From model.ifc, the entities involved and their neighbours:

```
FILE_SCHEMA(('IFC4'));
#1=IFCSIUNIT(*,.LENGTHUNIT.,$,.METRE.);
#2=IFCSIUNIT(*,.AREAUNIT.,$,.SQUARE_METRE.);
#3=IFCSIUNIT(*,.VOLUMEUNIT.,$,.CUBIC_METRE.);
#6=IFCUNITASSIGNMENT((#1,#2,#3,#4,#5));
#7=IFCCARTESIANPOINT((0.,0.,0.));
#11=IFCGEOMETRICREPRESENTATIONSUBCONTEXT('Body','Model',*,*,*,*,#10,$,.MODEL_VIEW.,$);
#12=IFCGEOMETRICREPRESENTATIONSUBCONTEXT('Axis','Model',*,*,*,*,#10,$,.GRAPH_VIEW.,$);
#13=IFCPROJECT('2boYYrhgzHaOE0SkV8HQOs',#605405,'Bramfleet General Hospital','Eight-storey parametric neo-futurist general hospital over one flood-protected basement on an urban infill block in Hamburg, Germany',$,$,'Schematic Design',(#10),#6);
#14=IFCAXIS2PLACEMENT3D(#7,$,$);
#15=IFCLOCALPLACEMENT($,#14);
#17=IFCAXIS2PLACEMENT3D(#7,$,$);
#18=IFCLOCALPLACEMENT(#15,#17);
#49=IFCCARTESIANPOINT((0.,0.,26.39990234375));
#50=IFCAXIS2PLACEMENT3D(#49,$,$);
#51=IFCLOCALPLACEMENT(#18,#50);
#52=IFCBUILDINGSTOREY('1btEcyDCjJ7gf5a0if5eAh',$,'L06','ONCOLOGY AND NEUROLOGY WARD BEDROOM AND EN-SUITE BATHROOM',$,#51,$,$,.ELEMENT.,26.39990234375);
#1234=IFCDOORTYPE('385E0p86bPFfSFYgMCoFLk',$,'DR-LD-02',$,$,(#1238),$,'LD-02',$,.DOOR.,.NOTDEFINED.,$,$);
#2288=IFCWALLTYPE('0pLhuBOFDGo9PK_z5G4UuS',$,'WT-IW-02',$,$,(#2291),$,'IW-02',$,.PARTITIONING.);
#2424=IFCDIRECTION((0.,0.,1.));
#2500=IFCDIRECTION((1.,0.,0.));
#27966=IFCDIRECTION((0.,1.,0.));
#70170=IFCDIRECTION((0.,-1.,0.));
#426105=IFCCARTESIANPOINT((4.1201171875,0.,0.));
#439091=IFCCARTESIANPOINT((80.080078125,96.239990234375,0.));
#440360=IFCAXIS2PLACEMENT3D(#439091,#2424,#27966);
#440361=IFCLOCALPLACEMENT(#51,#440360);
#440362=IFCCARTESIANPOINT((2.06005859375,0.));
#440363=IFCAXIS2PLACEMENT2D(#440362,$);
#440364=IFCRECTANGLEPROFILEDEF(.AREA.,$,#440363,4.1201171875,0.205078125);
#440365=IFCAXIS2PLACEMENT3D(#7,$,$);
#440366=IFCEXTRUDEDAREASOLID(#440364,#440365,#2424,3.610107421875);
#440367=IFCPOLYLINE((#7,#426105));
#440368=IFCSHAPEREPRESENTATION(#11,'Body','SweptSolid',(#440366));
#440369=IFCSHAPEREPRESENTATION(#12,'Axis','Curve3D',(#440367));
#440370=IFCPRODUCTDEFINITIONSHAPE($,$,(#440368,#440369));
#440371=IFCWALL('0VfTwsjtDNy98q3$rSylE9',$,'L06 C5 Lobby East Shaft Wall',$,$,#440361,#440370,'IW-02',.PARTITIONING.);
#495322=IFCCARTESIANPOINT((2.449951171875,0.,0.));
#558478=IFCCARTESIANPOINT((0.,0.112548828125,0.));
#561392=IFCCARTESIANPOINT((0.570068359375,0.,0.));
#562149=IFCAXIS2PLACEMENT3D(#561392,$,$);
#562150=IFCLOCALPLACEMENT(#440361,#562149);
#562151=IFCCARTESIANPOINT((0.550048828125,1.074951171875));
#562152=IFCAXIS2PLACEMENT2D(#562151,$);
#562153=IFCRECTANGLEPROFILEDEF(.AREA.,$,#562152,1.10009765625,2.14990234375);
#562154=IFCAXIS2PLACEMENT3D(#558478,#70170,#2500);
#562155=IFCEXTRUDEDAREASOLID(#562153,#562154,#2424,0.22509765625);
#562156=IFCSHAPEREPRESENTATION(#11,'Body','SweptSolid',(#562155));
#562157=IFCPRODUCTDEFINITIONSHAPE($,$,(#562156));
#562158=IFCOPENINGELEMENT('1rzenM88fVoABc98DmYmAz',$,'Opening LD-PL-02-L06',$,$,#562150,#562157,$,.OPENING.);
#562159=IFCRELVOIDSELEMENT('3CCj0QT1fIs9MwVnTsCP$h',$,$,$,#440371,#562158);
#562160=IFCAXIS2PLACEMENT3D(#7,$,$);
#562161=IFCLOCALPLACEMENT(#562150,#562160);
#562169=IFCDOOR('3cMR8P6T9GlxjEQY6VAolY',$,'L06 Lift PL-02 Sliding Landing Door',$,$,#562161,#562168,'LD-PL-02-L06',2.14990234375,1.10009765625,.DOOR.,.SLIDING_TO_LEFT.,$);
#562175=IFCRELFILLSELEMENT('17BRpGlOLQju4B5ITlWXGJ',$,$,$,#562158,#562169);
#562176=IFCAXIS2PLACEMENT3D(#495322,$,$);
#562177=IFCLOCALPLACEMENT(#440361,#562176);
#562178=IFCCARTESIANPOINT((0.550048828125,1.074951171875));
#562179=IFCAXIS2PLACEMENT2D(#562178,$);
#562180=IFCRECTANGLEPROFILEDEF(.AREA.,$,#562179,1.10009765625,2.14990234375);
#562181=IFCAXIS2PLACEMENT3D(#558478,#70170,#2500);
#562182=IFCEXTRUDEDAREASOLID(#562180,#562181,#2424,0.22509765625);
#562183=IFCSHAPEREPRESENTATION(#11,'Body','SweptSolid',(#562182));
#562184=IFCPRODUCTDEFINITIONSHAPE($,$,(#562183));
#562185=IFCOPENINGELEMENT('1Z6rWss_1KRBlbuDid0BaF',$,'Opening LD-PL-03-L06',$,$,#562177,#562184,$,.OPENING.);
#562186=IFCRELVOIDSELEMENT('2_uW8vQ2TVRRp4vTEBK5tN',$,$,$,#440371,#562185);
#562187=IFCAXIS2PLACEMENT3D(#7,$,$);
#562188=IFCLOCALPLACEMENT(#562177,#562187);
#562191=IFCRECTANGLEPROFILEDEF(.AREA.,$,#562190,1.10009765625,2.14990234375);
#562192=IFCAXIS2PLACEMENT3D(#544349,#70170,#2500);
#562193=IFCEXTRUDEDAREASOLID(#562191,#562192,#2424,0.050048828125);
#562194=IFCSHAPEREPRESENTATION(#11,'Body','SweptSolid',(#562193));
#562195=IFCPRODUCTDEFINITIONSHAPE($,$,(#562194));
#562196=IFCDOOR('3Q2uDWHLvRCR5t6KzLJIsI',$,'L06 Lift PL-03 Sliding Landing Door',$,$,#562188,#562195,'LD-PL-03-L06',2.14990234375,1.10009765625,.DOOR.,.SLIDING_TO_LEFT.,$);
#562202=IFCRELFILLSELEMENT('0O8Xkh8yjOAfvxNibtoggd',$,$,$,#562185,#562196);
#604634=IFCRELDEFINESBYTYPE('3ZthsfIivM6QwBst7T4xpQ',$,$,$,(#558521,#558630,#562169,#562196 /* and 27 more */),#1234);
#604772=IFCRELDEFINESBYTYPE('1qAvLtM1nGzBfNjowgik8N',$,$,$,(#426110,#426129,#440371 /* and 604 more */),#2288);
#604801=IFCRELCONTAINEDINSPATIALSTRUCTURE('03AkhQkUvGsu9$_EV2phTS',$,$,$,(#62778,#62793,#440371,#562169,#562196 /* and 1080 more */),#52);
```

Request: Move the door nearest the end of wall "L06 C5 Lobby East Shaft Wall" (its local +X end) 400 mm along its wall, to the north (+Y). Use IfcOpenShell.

```python
import ifcopenshell
import ifcopenshell.api.geometry
import ifcopenshell.util.placement
import ifcopenshell.util.unit

model = ifcopenshell.open("model.ifc")
unit_scale = ifcopenshell.util.unit.calculate_unit_scale(model)

door = model.by_guid("3Q2uDWHLvRCR5t6KzLJIsI")
opening = door.FillsVoids[0].RelatingOpeningElement
wall = opening.VoidsElements[0].RelatingBuildingElement

wall_matrix = ifcopenshell.util.placement.get_local_placement(wall.ObjectPlacement)
shift = wall_matrix[:3, 0] * 0.4 / unit_scale
before = ifcopenshell.util.placement.get_local_placement(door.ObjectPlacement)[:3, 3].copy()

# The door is placed relative to its opening, so it follows when the opening moves.
matrix = ifcopenshell.util.placement.get_local_placement(opening.ObjectPlacement)
matrix[:3, 3] += shift
ifcopenshell.api.geometry.edit_object_placement(
    model, product=opening, matrix=matrix, is_si=False, should_transform_children=True
)

after = ifcopenshell.util.placement.get_local_placement(door.ObjectPlacement)[:3, 3]
print("door moved by", (after - before).round(3) + 0.0)

model.write("model_edited.ifc")
```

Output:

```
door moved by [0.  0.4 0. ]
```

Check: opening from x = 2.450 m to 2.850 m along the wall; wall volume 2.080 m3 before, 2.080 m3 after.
